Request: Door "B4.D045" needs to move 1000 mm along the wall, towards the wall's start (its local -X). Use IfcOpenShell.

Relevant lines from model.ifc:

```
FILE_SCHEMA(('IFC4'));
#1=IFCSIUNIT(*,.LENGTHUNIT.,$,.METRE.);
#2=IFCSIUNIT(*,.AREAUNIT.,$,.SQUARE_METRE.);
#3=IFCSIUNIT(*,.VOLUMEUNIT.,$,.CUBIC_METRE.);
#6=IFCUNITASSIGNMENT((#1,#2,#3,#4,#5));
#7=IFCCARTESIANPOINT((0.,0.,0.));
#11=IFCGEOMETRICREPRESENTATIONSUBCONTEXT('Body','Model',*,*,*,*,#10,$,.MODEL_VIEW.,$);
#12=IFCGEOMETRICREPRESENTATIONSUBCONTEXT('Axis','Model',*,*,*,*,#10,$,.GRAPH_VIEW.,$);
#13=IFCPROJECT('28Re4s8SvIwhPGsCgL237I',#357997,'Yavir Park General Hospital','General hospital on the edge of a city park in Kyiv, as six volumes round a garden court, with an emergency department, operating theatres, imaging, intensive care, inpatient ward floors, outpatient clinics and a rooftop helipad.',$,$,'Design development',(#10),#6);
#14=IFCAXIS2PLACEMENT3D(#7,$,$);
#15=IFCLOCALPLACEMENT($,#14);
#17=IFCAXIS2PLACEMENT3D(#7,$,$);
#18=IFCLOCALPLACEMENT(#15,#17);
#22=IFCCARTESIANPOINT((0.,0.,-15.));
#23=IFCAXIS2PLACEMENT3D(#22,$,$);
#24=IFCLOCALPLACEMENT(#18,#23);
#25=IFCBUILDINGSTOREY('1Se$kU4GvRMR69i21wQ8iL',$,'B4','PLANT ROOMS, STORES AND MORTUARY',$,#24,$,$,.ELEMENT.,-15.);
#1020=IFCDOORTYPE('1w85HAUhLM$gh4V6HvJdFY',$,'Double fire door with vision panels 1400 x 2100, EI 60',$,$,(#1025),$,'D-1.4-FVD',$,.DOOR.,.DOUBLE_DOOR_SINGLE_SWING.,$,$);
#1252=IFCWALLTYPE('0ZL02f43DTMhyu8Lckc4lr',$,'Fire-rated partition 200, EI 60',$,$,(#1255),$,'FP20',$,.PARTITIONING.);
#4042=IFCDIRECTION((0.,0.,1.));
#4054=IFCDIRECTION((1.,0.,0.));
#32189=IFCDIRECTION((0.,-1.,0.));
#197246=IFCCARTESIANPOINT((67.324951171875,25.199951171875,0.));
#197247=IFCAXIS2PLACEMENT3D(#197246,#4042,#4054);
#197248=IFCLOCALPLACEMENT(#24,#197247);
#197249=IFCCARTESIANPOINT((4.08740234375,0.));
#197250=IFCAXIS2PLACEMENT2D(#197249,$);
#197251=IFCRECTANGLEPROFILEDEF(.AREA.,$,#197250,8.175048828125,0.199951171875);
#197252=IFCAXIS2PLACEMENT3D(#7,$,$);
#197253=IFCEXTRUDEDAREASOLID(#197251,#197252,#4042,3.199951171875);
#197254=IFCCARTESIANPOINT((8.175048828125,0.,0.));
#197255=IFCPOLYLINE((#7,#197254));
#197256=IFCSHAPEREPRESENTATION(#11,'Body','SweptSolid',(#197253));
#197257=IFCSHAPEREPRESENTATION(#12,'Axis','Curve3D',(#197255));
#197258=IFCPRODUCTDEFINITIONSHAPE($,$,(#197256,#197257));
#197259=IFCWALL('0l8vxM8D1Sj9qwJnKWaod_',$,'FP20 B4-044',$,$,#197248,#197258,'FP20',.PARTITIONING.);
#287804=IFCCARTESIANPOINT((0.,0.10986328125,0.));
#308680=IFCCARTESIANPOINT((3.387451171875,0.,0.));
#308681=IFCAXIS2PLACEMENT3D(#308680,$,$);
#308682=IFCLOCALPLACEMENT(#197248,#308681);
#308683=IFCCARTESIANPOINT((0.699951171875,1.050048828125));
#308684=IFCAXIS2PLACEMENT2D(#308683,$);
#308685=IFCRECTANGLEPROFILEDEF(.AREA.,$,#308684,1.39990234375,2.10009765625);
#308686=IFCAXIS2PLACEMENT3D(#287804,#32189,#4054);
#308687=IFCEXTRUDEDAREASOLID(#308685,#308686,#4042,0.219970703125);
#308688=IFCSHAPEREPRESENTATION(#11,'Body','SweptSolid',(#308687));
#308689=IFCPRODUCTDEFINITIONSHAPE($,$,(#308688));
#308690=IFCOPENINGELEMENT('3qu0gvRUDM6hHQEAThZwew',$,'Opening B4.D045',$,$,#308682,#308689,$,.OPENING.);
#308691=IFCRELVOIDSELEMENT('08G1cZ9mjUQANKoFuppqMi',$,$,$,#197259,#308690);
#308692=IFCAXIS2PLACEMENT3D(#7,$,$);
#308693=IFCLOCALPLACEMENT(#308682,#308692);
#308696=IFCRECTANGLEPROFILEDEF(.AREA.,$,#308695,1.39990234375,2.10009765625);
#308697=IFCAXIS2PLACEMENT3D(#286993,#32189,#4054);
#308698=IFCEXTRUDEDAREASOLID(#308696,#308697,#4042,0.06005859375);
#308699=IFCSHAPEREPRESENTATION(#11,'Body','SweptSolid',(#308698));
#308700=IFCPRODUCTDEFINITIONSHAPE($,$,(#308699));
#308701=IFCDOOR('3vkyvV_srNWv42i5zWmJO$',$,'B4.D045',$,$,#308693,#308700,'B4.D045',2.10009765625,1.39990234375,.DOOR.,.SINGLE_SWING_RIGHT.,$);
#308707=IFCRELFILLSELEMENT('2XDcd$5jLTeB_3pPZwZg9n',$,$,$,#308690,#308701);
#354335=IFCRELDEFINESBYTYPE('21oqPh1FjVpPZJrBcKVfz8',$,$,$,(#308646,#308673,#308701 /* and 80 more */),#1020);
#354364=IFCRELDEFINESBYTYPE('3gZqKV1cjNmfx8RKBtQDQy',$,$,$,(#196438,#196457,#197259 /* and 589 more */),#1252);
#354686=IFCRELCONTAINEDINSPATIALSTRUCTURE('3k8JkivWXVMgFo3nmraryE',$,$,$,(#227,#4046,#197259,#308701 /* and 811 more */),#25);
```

```python
import ifcopenshell
import ifcopenshell.api.geometry
import ifcopenshell.util.placement
import ifcopenshell.util.unit

model = ifcopenshell.open("model.ifc")
unit_scale = ifcopenshell.util.unit.calculate_unit_scale(model)

door = model.by_id(308701)
opening = door.FillsVoids[0].RelatingOpeningElement
wall = opening.VoidsElements[0].RelatingBuildingElement

wall_matrix = ifcopenshell.util.placement.get_local_placement(wall.ObjectPlacement)
shift = wall_matrix[:3, 0] * -1 / unit_scale
before = ifcopenshell.util.placement.get_local_placement(door.ObjectPlacement)[:3, 3].copy()

# The door is placed relative to its opening, so it follows when the opening moves.
matrix = ifcopenshell.util.placement.get_local_placement(opening.ObjectPlacement)
matrix[:3, 3] += shift
ifcopenshell.api.geometry.edit_object_placement(
    model, product=opening, matrix=matrix, is_si=False, should_transform_children=True
)

after = ifcopenshell.util.placement.get_local_placement(door.ObjectPlacement)[:3, 3]
print("door moved by", (after - before).round(3) + 0.0)

model.write("model-out.ifc")
```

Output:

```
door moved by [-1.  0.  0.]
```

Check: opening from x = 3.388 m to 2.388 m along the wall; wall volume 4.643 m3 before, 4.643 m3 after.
